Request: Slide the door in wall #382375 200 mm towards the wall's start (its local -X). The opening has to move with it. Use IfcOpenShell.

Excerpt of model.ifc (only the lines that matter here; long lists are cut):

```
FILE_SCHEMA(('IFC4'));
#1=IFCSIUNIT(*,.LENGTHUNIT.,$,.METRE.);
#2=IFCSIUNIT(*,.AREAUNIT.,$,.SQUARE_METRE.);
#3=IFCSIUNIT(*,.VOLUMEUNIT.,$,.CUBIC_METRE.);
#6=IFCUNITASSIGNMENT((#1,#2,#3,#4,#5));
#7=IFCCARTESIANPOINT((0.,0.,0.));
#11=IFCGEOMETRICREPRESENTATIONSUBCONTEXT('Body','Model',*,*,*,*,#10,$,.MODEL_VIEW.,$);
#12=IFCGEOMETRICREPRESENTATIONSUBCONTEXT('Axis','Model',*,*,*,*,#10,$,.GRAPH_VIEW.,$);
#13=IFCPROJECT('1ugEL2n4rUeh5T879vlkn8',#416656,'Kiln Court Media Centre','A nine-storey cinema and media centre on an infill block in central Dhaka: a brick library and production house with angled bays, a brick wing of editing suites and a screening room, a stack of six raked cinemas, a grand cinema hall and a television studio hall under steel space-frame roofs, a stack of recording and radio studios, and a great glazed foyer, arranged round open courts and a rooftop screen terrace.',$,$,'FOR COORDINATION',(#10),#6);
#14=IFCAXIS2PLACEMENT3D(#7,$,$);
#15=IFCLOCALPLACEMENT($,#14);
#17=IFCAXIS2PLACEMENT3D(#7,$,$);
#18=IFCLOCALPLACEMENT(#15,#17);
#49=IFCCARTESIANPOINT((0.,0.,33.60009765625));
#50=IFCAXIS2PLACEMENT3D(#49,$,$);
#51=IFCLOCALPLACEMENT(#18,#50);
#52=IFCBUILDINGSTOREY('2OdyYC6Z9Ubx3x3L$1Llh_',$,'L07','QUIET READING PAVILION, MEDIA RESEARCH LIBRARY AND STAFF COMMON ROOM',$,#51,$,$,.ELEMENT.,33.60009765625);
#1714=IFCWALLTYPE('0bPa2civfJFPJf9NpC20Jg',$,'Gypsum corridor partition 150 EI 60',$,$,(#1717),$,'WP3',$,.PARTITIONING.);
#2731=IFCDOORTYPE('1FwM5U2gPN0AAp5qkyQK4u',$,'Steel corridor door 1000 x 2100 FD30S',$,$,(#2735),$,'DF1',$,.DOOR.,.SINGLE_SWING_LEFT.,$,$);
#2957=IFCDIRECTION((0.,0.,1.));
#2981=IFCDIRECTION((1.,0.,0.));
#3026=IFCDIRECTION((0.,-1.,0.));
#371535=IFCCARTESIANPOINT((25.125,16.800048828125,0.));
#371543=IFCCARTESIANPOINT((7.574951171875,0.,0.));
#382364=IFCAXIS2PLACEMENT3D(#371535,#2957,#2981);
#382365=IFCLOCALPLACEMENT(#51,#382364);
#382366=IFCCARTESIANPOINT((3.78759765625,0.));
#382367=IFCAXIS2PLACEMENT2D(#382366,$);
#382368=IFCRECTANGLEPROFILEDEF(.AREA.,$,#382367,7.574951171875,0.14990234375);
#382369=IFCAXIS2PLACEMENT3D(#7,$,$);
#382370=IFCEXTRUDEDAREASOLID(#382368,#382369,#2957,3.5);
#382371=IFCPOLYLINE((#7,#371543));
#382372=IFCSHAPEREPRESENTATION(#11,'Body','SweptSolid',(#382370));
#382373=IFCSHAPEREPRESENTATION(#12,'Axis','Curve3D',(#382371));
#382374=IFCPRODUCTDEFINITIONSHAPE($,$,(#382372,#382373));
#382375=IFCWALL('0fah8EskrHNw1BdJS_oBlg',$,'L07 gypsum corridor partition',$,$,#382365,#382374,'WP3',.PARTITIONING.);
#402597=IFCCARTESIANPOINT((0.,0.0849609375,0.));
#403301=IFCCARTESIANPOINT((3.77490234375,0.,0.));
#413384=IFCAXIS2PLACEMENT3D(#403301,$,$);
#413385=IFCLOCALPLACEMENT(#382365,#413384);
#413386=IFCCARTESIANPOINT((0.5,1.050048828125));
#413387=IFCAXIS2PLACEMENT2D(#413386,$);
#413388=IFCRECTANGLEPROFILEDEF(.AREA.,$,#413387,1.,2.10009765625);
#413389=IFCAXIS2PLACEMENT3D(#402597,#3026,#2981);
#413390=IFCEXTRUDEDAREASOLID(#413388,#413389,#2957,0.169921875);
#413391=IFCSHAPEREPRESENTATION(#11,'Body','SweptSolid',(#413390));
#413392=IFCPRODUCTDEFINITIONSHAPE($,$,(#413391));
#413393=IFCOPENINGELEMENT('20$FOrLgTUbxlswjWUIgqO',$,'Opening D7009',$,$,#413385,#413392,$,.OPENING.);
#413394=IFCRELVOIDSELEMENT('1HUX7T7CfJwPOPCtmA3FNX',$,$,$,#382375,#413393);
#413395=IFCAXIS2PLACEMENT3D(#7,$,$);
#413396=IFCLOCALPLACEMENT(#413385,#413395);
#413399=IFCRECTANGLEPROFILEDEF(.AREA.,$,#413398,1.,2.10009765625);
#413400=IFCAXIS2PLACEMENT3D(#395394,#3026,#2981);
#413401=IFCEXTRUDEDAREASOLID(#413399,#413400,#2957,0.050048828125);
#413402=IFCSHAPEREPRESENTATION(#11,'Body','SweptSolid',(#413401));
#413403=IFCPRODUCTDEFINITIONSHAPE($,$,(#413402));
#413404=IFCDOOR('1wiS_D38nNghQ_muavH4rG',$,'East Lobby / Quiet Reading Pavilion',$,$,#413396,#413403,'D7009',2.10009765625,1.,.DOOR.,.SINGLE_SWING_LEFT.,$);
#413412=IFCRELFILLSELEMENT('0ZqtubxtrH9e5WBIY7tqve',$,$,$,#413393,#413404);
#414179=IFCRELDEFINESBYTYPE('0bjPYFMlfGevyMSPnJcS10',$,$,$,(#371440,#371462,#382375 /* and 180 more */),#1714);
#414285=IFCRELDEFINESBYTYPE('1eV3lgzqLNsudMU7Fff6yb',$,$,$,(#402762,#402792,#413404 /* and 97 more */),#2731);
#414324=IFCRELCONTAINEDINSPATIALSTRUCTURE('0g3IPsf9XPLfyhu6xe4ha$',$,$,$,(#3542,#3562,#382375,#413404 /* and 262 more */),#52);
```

```python
import ifcopenshell
import ifcopenshell.api.geometry
import ifcopenshell.util.placement

model = ifcopenshell.open("model.ifc")

door = model.by_guid("1wiS_D38nNghQ_muavH4rG")
opening = door.FillsVoids[0].RelatingOpeningElement
wall = opening.VoidsElements[0].RelatingBuildingElement

wall_matrix = ifcopenshell.util.placement.get_local_placement(wall.ObjectPlacement)
shift = wall_matrix[:3, 0] * -0.2
before = ifcopenshell.util.placement.get_local_placement(door.ObjectPlacement)[:3, 3].copy()

# The door is placed relative to its opening, so it follows when the opening moves.
matrix = ifcopenshell.util.placement.get_local_placement(opening.ObjectPlacement)
matrix[:3, 3] += shift
ifcopenshell.api.geometry.edit_object_placement(
    model, product=opening, matrix=matrix, is_si=False, should_transform_children=True
)

after = ifcopenshell.util.placement.get_local_placement(door.ObjectPlacement)[:3, 3]
print("door moved by", (after - before).round(3) + 0.0)

model.write("model_v2.ifc")
```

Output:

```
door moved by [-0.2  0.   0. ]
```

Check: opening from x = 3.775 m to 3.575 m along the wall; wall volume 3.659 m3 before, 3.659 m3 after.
